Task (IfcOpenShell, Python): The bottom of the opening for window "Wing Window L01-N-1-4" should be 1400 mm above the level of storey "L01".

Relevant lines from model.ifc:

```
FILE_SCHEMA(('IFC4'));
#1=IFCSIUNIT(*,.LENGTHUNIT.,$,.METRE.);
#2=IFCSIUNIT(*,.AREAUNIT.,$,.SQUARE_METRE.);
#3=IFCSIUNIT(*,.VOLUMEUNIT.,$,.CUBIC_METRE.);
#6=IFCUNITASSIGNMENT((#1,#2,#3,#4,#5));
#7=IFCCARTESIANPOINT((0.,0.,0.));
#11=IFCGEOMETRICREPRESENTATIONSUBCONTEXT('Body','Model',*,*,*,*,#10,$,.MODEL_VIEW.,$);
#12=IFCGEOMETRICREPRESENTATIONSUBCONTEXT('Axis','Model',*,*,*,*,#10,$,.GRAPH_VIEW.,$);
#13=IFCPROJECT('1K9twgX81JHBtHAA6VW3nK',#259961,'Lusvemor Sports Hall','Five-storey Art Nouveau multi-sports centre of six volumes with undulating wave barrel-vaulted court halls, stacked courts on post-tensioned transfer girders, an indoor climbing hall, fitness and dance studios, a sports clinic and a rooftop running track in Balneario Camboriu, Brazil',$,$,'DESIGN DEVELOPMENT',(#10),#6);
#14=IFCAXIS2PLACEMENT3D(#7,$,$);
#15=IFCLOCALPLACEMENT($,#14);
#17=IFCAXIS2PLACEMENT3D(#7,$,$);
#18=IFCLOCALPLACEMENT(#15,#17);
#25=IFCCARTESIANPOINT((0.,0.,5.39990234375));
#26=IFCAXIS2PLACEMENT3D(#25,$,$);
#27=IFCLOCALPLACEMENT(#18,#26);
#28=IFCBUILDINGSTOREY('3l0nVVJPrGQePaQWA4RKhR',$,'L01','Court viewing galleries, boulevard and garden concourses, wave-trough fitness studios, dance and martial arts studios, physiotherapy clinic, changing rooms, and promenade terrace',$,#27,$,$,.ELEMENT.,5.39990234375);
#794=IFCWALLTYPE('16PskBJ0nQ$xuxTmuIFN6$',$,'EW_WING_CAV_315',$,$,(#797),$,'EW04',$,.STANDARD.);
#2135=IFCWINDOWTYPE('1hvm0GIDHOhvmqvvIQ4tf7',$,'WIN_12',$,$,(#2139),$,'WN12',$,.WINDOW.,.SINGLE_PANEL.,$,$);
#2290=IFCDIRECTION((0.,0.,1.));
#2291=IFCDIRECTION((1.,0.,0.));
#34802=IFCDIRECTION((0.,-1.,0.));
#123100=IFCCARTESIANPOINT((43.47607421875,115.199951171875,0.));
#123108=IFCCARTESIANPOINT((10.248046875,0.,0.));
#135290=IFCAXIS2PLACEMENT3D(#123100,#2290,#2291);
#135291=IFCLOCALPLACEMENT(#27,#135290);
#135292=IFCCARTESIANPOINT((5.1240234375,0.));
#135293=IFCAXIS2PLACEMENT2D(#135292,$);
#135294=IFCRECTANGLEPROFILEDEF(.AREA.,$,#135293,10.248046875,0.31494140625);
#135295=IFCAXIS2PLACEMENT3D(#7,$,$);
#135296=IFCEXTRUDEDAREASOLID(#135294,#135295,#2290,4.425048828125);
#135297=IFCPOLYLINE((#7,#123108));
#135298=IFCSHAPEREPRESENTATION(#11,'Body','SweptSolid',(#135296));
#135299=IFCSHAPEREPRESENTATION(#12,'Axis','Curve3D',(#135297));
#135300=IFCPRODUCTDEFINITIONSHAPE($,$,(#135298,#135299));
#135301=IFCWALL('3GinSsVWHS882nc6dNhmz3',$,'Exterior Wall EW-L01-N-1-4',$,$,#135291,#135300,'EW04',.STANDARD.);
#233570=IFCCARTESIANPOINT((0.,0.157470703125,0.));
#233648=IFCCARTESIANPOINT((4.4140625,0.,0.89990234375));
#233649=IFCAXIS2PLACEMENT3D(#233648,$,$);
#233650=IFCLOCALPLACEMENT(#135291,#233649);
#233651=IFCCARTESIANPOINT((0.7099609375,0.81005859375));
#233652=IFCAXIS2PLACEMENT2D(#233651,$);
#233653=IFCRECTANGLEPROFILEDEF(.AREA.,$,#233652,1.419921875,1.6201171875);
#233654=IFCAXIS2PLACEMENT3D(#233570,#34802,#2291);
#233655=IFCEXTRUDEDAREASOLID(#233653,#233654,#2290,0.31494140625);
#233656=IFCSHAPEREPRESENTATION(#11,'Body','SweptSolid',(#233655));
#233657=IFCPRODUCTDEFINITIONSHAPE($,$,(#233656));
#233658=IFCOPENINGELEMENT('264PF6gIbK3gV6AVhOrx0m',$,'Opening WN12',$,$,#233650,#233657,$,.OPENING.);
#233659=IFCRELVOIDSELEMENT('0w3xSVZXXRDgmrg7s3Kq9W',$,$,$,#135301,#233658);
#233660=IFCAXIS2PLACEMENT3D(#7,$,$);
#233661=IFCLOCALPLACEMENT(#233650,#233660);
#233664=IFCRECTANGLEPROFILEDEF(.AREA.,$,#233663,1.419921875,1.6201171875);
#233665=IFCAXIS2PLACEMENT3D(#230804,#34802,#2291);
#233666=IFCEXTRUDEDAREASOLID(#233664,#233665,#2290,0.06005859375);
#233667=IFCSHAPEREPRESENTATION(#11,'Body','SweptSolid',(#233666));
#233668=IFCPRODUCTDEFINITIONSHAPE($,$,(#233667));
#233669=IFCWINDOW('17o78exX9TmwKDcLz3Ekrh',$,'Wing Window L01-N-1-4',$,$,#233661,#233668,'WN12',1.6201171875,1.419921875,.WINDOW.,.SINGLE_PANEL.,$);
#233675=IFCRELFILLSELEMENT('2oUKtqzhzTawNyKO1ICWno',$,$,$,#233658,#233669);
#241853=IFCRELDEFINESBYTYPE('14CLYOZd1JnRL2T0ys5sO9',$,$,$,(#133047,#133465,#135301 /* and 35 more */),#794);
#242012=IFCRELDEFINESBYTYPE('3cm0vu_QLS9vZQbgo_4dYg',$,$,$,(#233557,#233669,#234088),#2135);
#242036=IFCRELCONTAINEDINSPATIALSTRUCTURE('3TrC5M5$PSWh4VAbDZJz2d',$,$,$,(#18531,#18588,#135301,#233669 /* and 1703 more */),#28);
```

```python
import numpy as np
import ifcopenshell
import ifcopenshell.api.geometry
import ifcopenshell.geom
import ifcopenshell.util.element
import ifcopenshell.util.placement
import ifcopenshell.util.shape
import ifcopenshell.util.unit

model = ifcopenshell.open("model.ifc")
unit_scale = ifcopenshell.util.unit.calculate_unit_scale(model)

window = model.by_guid("17o78exX9TmwKDcLz3Ekrh")
opening = window.FillsVoids[0].RelatingOpeningElement
storey = ifcopenshell.util.element.get_container(window, ifc_class="IfcBuildingStorey")
level = ifcopenshell.util.placement.get_local_placement(storey.ObjectPlacement)[2, 3]

# The opening's origin need not be at the sill, so measure its lowest point.
shape = ifcopenshell.geom.create_shape(ifcopenshell.geom.settings(), opening)
bottom = ifcopenshell.util.shape.get_shape_bottom_elevation(shape, shape.geometry) / unit_scale
dz = level + 1.4 / unit_scale - bottom

shift = np.array([0.0, 0.0, dz])
# The window is placed relative to its opening, so it follows when the opening moves.
matrix = ifcopenshell.util.placement.get_local_placement(opening.ObjectPlacement)
matrix[:3, 3] += shift
ifcopenshell.api.geometry.edit_object_placement(
    model, product=opening, matrix=matrix, is_si=False, should_transform_children=True
)

print(f"moved by {dz * unit_scale:+.3f} m")

model.write("model_updated.ifc")
```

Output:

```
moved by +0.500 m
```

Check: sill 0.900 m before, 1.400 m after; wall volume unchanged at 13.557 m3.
